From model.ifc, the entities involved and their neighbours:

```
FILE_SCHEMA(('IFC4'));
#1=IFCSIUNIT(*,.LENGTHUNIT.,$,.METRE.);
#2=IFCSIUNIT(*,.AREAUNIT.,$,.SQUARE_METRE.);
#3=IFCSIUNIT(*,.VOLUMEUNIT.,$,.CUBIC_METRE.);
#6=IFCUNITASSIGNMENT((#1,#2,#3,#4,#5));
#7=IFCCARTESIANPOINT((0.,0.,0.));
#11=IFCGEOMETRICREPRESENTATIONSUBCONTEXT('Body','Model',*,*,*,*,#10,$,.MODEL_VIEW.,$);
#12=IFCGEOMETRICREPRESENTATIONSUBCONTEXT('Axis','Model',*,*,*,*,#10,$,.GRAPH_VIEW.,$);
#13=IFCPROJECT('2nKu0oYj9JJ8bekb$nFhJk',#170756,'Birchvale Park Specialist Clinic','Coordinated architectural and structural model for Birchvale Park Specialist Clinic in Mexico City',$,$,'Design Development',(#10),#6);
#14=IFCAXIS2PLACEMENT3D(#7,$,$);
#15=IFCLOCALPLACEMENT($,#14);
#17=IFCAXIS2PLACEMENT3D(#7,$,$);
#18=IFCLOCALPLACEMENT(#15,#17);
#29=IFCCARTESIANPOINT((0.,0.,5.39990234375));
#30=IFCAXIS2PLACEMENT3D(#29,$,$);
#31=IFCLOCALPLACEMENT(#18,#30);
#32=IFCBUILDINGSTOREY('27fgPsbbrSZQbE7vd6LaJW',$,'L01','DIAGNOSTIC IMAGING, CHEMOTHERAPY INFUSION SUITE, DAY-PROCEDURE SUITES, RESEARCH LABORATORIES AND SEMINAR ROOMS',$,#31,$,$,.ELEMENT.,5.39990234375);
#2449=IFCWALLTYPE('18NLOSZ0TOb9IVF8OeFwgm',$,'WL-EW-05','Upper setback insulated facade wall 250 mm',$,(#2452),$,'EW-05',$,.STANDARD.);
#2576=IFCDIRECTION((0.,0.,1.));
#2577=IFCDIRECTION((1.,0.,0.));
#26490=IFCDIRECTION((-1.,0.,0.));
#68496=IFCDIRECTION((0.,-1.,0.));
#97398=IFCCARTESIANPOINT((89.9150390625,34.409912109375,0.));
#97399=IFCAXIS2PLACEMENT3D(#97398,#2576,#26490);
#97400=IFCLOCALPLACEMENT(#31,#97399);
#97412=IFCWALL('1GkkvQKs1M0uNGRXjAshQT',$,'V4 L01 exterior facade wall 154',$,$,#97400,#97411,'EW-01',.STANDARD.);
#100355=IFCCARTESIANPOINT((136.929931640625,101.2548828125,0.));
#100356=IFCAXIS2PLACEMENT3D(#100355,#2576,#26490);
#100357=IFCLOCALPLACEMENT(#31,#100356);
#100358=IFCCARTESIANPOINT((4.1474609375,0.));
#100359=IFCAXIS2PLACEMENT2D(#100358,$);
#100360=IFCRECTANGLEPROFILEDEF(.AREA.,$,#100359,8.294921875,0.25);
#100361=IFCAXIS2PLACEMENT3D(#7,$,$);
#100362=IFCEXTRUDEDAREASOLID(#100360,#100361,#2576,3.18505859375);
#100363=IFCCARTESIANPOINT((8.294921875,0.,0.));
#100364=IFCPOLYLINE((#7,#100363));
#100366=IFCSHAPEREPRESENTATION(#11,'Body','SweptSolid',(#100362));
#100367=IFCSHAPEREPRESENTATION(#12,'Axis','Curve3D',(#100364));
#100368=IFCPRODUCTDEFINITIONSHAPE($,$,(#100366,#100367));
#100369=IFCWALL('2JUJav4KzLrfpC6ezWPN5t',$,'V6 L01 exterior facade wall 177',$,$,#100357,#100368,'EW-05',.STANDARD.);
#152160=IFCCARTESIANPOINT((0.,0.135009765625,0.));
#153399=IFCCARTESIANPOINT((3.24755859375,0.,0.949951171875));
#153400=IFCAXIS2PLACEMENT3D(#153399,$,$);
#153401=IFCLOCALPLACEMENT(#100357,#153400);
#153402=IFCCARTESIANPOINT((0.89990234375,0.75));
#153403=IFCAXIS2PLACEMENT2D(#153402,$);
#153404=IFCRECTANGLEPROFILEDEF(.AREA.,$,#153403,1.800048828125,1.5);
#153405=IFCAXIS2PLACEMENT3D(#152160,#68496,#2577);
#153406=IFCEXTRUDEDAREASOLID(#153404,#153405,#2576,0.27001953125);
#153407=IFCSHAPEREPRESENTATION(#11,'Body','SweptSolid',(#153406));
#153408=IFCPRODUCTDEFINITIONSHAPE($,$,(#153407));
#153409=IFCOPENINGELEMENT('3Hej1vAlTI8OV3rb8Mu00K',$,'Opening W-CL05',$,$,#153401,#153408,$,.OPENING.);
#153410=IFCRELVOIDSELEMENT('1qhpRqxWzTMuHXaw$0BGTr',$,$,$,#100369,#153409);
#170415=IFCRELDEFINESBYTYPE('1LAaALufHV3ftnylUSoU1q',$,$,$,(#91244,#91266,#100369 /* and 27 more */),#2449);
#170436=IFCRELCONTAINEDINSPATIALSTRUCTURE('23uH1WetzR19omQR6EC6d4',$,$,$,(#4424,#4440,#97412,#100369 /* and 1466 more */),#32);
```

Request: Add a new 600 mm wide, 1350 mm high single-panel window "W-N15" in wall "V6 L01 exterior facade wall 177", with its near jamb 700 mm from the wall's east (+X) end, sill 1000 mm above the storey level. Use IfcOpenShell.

```python
import numpy as np
import ifcopenshell
import ifcopenshell.api.feature
import ifcopenshell.api.geometry
import ifcopenshell.api.root
import ifcopenshell.api.spatial
import ifcopenshell.geom
import ifcopenshell.util.element
import ifcopenshell.util.placement
import ifcopenshell.util.representation
import ifcopenshell.util.shape
import ifcopenshell.util.unit

model = ifcopenshell.open("model.ifc")
unit_scale = ifcopenshell.util.unit.calculate_unit_scale(model)
settings = ifcopenshell.geom.settings()


def volume(element):
    """Net volume in cubic metres, openings subtracted."""
    shape = ifcopenshell.geom.create_shape(settings, element)
    return ifcopenshell.util.shape.get_volume(shape.geometry)


wall = model.by_guid("2JUJav4KzLrfpC6ezWPN5t")
storey = ifcopenshell.util.element.get_container(wall, ifc_class="IfcBuildingStorey")
context = ifcopenshell.util.representation.get_context(model, "Model", "Body", "MODEL_VIEW")
before = volume(wall)

width, height, from_end, sill = 0.6, 1.35, 0.7, 1  # metres

# The wall runs along its own X axis, and the end named is its -X end.
wall_shape = ifcopenshell.geom.create_shape(settings, wall)
x, y, z = ifcopenshell.util.shape.get_vertices(wall_shape.geometry).T
start = x.min() + from_end
face, thickness = float(y.min()), float(y.max() - y.min())
wall_matrix = ifcopenshell.util.placement.get_local_placement(wall.ObjectPlacement)
level = ifcopenshell.util.placement.get_local_placement(storey.ObjectPlacement)[2, 3]


def in_wall(x, y):
    """Placement at x, y metres in the wall's axes, at sill height."""
    matrix = wall_matrix.copy()
    matrix[:, 3] = wall_matrix @ np.array([x / unit_scale, y / unit_scale, 0.0, 1.0])
    matrix[2, 3] = level + sill / unit_scale
    return matrix


# Opening: a box that overshoots both wall faces by 50 mm.
opening = ifcopenshell.api.root.create_entity(model, ifc_class="IfcOpeningElement", predefined_type="OPENING")
box = ifcopenshell.api.geometry.add_wall_representation(
    model, context=context, length=width, height=height, thickness=thickness + 0.1
)
ifcopenshell.api.geometry.assign_representation(model, product=opening, representation=box)
ifcopenshell.api.geometry.edit_object_placement(model, product=opening, matrix=in_wall(start, face - 0.05), is_si=False)
ifcopenshell.api.feature.add_feature(model, feature=opening, element=wall)

window = ifcopenshell.api.root.create_entity(model, ifc_class="IfcWindow", name="W-N15", predefined_type="WINDOW")
window.OverallWidth, window.OverallHeight = width / unit_scale, height / unit_scale
window.PartitioningType = "SINGLE_PANEL"
body = ifcopenshell.api.geometry.add_window_representation(
    model,
    context=context,
    overall_width=window.OverallWidth,
    overall_height=window.OverallHeight,
    partition_type="SINGLE_PANEL",
)
ifcopenshell.api.geometry.assign_representation(model, product=window, representation=body)
ifcopenshell.api.spatial.assign_container(model, products=[window], relating_structure=storey)
ifcopenshell.api.feature.add_filling(model, opening=opening, element=window)

# Centre the window in the wall's thickness.
ifcopenshell.api.geometry.edit_object_placement(model, product=window, matrix=in_wall(start, face), is_si=False)
window_shape = ifcopenshell.geom.create_shape(settings, window)
depth = ifcopenshell.util.shape.get_vertices(window_shape.geometry)[:, 1]
offset = face + thickness / 2 - (depth.min() + depth.max()) / 2
ifcopenshell.api.geometry.edit_object_placement(model, product=window, matrix=in_wall(start, offset), is_si=False)

after = volume(wall)

print(f"wall volume {before:.3f} -> {after:.3f} m3")

model.write("model_updated.ifc")
```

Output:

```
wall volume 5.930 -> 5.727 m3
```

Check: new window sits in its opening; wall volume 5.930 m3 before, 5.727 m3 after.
